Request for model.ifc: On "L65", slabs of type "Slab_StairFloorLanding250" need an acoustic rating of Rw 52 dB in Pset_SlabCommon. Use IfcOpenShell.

First a look at what the model holds.

```python
import ifcopenshell
import ifcopenshell.util.element

model = ifcopenshell.open("model.ifc")
print(model.schema)
storey = next(s for s in model.by_type("IfcBuildingStorey") if s.Name == "L65")
slabs = [e for e in ifcopenshell.util.element.get_decomposition(storey) if e.is_a("IfcSlab")]
seen = {}
for e in slabs:
    element_type = ifcopenshell.util.element.get_type(e)
    key = (element_type.Name if element_type != e and element_type else None, ifcopenshell.util.element.get_pset(e, "Pset_SlabCommon", "AcousticRating"))
    seen[key] = seen.get(key, 0) + 1
for (name, value), count in sorted(seen.items(), key=str):
    print(count, "x", name, "|", value)
```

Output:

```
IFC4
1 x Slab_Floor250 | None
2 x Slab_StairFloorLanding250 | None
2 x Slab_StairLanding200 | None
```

```python
import ifcopenshell
import ifcopenshell.api.pset
import ifcopenshell.util.element

model = ifcopenshell.open("model.ifc")

storey = next(s for s in model.by_type("IfcBuildingStorey") if s.Name == "L65")
slabs = [e for e in ifcopenshell.util.element.get_decomposition(storey) if e.is_a("IfcSlab")]

count = 0
for e in slabs:
    element_type = ifcopenshell.util.element.get_type(e)
    if element_type in (None, e) or element_type.Name != "Slab_StairFloorLanding250":
        continue
    found = ifcopenshell.util.element.get_pset(e, "Pset_SlabCommon", should_inherit=False)
    if found:
        pset = model.by_id(found["id"])
        if len(ifcopenshell.util.element.get_elements_by_pset(pset)) > 1:
            pset = ifcopenshell.api.pset.unshare_pset(model, products=[e], pset=pset)[0]
    else:
        pset = ifcopenshell.api.pset.add_pset(model, product=e, name="Pset_SlabCommon")
    ifcopenshell.api.pset.edit_pset(model, pset=pset, properties={"AcousticRating": "Rw 52 dB"})
    count += 1

print(count, "slabs updated")

model.write("model_rev.ifc")
```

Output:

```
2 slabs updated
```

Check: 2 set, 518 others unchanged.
